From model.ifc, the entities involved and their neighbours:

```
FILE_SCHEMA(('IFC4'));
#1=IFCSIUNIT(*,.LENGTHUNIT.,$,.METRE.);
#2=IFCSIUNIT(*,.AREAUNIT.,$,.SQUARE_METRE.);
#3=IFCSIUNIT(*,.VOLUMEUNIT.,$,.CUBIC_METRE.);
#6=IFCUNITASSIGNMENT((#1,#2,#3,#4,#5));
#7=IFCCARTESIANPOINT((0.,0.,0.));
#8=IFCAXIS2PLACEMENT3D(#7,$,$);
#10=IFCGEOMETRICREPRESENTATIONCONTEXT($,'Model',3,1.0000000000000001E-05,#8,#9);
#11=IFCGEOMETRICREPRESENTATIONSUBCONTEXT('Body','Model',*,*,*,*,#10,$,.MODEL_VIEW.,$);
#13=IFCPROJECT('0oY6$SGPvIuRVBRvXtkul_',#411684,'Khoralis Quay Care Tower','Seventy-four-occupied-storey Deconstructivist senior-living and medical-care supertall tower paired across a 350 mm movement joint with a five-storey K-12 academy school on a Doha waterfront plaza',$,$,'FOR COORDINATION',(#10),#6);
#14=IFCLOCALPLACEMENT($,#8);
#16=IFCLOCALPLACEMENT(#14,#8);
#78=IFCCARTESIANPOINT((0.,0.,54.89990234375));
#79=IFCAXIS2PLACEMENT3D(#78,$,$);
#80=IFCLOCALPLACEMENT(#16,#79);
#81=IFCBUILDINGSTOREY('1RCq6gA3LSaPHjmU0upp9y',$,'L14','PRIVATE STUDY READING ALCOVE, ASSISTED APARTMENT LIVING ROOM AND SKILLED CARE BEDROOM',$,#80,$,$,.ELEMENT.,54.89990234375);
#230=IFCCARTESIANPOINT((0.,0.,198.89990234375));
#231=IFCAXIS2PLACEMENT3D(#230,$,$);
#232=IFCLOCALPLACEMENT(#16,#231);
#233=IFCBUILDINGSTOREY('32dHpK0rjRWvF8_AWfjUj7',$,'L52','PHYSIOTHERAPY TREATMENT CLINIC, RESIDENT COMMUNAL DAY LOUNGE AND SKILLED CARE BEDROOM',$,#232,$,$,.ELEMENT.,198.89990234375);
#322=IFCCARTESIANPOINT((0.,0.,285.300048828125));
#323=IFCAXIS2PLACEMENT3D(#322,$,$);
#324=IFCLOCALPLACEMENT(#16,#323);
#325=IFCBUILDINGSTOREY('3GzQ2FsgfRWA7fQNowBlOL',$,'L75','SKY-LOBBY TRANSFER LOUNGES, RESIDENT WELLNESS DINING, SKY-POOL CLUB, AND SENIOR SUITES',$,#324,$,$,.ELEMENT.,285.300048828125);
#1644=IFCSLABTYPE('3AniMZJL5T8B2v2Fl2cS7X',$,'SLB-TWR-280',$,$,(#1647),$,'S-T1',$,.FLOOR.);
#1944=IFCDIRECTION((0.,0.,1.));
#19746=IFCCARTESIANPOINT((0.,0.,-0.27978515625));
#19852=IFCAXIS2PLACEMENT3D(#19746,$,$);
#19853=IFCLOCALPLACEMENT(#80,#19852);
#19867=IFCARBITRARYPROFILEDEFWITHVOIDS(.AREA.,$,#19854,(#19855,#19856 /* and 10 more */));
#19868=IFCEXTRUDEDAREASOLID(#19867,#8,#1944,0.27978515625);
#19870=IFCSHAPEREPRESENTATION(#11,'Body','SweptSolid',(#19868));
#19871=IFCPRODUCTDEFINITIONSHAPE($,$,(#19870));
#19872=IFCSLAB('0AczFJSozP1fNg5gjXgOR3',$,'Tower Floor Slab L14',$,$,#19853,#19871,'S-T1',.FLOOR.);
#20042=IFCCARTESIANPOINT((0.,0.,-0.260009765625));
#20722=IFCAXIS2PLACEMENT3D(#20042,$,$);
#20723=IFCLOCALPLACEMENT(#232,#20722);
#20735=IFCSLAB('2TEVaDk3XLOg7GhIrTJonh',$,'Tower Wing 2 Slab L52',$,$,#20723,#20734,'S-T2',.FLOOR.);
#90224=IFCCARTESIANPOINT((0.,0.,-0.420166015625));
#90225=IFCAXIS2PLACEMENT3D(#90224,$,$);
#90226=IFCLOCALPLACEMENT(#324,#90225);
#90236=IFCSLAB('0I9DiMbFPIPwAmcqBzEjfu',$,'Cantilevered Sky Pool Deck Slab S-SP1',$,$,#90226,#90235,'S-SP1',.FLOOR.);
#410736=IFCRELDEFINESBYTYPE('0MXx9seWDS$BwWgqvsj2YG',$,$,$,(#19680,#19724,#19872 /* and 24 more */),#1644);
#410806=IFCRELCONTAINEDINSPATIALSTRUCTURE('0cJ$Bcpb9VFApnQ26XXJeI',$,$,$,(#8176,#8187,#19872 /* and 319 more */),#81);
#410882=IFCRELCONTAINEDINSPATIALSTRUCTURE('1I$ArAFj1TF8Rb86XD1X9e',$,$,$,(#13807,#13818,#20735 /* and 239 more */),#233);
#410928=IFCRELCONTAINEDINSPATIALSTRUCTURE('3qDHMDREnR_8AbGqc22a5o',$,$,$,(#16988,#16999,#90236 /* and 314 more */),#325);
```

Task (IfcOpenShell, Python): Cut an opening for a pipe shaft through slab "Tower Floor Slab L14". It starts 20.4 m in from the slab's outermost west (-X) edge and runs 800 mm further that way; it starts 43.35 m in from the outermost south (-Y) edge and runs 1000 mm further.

```python
import numpy as np
import ifcopenshell
import ifcopenshell.api.feature
import ifcopenshell.api.geometry
import ifcopenshell.api.root
import ifcopenshell.geom
import ifcopenshell.util.placement
import ifcopenshell.util.representation
import ifcopenshell.util.shape
import ifcopenshell.util.unit

model = ifcopenshell.open("model.ifc")
unit_scale = ifcopenshell.util.unit.calculate_unit_scale(model)
settings = ifcopenshell.geom.settings()


def volume(element):
    """Net volume in cubic metres, openings subtracted."""
    shape = ifcopenshell.geom.create_shape(settings, element)
    return ifcopenshell.util.shape.get_volume(shape.geometry)


slab = model.by_guid("0AczFJSozP1fNg5gjXgOR3")
before = volume(slab)

# Extent in the slab's own axes, in metres. The edges named are its -X and -Y sides.
slab_shape = ifcopenshell.geom.create_shape(settings, slab)
vertices = ifcopenshell.util.shape.get_vertices(slab_shape.geometry)
x_min, y_min, bottom = vertices.min(axis=0)
top = vertices[:, 2].max()

opening = ifcopenshell.api.root.create_entity(model, ifc_class="IfcOpeningElement", name="Pipe shaft opening", predefined_type="OPENING")
context = ifcopenshell.util.representation.get_context(model, "Model", "Body", "MODEL_VIEW")
width, depth = 0.8, 1
outline = [(0.0, 0.0), (width, 0.0), (width, depth), (0.0, depth), (0.0, 0.0)]
# Overshoot both faces by 50 mm so the cut is clean.
shape = ifcopenshell.api.geometry.add_slab_representation(
    model, context=context, depth=top - bottom + 0.1, polyline=outline
)
ifcopenshell.api.geometry.assign_representation(model, product=opening, representation=shape)

matrix = ifcopenshell.util.placement.get_local_placement(slab.ObjectPlacement)
matrix[:, 3] = matrix @ np.append(np.array([x_min + 20.4, y_min + 43.35, bottom - 0.05]) / unit_scale, 1.0)
ifcopenshell.api.geometry.edit_object_placement(model, product=opening, matrix=matrix, is_si=False)
ifcopenshell.api.feature.add_feature(model, feature=opening, element=slab)

after = volume(slab)

print(f"slab volume {before:.3f} -> {after:.3f} m3")

model.write("model-out.ifc")
```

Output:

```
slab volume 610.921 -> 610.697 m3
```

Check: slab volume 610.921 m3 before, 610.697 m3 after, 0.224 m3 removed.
